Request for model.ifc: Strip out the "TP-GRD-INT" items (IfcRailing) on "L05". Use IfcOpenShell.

First a look at what the model holds.

```python
import ifcopenshell
import ifcopenshell.util.element

model = ifcopenshell.open("model.ifc")
print(model.schema)
storey = next(s for s in model.by_type("IfcBuildingStorey") if s.Name == "L05")
railings = [e for e in ifcopenshell.util.element.get_decomposition(storey) if e.is_a("IfcRailing")]
seen = {}
for e in railings:
    element_type = ifcopenshell.util.element.get_type(e)
    name = element_type.Name if element_type not in (None, e) else None
    seen[name] = seen.get(name, 0) + 1
for name, count in sorted(seen.items(), key=str):
    print(count, "x", name)
```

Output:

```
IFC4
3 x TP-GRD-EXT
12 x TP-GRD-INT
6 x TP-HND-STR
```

```python
import ifcopenshell
import ifcopenshell.api.root
import ifcopenshell.util.element

model = ifcopenshell.open("model.ifc")

storey = next(s for s in model.by_type("IfcBuildingStorey") if s.Name == "L05")
railings = [e for e in ifcopenshell.util.element.get_decomposition(storey) if e.is_a("IfcRailing")]
targets = [e for e in railings if (t := ifcopenshell.util.element.get_type(e)) not in (None, e) and t.Name == "TP-GRD-INT"]

for e in targets:
    ifcopenshell.api.root.remove_product(model, product=e)
print(len(targets), "removed")

model.write("model_updated.ifc")
```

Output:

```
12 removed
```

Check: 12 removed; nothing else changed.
